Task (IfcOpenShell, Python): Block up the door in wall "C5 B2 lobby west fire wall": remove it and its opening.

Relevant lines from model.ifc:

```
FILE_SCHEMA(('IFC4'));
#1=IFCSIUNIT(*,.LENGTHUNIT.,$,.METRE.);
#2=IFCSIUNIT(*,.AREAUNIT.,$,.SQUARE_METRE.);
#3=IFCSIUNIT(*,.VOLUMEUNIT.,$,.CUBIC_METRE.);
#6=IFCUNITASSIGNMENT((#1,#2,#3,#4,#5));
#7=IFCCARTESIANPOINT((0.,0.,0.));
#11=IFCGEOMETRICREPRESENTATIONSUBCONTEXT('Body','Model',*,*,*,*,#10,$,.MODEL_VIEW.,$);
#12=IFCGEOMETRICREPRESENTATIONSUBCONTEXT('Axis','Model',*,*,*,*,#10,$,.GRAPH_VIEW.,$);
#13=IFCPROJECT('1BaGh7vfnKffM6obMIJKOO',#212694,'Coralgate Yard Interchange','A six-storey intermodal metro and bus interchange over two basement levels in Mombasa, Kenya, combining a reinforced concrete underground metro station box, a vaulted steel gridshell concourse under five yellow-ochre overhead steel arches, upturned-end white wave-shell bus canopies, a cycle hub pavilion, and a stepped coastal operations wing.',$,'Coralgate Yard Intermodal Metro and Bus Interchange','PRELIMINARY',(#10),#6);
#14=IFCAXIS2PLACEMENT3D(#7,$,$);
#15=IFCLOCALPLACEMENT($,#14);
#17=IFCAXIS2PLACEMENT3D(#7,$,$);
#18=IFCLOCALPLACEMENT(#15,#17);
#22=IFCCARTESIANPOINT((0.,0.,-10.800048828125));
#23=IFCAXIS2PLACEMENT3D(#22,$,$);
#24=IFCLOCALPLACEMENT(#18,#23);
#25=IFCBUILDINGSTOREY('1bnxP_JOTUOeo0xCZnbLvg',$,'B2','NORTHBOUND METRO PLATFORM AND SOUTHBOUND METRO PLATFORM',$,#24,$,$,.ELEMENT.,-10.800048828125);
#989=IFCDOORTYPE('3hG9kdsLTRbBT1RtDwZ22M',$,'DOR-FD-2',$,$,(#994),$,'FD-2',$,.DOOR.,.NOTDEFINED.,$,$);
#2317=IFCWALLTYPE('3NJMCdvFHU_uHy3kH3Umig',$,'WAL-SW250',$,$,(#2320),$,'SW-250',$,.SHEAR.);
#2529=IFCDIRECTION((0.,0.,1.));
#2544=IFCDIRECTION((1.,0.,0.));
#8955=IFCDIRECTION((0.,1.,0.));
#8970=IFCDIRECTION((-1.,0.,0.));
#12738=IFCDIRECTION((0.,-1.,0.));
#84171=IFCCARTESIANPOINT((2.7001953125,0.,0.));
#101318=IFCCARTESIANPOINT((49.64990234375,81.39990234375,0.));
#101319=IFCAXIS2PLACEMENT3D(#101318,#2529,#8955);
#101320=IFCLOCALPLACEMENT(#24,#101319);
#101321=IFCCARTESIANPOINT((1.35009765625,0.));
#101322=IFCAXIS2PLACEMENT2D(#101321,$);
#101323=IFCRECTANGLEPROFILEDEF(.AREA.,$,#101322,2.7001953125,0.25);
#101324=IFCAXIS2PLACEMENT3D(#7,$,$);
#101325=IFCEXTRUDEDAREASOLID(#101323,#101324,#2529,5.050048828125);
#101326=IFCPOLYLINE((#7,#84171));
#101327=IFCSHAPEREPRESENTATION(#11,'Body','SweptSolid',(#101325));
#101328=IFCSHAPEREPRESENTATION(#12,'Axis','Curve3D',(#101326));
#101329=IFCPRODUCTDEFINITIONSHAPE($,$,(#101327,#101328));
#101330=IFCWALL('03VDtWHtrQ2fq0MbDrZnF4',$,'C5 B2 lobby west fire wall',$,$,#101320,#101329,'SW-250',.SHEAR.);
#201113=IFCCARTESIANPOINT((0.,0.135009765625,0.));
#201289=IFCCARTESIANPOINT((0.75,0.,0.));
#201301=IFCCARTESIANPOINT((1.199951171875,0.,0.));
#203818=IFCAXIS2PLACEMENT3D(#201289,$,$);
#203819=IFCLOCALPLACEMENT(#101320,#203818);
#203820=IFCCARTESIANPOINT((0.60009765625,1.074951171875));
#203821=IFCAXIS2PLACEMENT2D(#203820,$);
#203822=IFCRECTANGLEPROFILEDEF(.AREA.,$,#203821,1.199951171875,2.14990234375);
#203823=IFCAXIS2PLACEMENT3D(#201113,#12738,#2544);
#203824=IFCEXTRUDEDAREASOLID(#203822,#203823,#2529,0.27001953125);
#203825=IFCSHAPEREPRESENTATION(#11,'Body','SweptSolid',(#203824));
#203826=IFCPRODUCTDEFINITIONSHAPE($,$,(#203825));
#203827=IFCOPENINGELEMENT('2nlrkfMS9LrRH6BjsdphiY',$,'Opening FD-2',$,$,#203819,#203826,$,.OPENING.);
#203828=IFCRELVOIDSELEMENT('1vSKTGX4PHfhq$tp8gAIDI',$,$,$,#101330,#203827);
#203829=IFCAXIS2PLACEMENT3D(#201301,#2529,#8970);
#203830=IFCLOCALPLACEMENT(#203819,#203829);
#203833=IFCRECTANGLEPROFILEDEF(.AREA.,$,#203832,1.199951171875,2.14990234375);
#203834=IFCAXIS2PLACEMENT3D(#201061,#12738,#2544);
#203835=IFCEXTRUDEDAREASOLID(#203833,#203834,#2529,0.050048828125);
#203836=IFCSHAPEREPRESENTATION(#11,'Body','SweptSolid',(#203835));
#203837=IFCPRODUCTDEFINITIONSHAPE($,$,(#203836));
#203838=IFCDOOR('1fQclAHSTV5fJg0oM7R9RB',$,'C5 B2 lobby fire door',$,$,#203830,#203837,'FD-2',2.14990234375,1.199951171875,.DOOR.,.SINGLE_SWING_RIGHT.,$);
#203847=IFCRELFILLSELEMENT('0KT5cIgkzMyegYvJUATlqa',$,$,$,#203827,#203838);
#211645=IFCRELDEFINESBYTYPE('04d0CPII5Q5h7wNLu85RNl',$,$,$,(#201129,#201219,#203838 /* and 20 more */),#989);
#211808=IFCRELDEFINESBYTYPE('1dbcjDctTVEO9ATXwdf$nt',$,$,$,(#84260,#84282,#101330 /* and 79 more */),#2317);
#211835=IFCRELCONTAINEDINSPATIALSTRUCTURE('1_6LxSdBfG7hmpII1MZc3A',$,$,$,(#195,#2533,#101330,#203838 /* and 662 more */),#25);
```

```python
import ifcopenshell
import ifcopenshell.api.feature
import ifcopenshell.api.root
import ifcopenshell.geom
import ifcopenshell.util.shape

model = ifcopenshell.open("model.ifc")
settings = ifcopenshell.geom.settings()


def volume(element):
    """Net volume in cubic metres, openings subtracted."""
    shape = ifcopenshell.geom.create_shape(settings, element)
    return ifcopenshell.util.shape.get_volume(shape.geometry)


door = model.by_id(203838)
opening = door.FillsVoids[0].RelatingOpeningElement
wall = opening.VoidsElements[0].RelatingBuildingElement
before = volume(wall)

ifcopenshell.api.root.remove_product(model, product=door)
ifcopenshell.api.feature.remove_feature(model, feature=opening)

after = volume(wall)

print(f"wall volume {before:.3f} -> {after:.3f} m3")

model.write("model-out.ifc")
```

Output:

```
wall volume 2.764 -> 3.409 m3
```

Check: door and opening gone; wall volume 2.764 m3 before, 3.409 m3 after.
